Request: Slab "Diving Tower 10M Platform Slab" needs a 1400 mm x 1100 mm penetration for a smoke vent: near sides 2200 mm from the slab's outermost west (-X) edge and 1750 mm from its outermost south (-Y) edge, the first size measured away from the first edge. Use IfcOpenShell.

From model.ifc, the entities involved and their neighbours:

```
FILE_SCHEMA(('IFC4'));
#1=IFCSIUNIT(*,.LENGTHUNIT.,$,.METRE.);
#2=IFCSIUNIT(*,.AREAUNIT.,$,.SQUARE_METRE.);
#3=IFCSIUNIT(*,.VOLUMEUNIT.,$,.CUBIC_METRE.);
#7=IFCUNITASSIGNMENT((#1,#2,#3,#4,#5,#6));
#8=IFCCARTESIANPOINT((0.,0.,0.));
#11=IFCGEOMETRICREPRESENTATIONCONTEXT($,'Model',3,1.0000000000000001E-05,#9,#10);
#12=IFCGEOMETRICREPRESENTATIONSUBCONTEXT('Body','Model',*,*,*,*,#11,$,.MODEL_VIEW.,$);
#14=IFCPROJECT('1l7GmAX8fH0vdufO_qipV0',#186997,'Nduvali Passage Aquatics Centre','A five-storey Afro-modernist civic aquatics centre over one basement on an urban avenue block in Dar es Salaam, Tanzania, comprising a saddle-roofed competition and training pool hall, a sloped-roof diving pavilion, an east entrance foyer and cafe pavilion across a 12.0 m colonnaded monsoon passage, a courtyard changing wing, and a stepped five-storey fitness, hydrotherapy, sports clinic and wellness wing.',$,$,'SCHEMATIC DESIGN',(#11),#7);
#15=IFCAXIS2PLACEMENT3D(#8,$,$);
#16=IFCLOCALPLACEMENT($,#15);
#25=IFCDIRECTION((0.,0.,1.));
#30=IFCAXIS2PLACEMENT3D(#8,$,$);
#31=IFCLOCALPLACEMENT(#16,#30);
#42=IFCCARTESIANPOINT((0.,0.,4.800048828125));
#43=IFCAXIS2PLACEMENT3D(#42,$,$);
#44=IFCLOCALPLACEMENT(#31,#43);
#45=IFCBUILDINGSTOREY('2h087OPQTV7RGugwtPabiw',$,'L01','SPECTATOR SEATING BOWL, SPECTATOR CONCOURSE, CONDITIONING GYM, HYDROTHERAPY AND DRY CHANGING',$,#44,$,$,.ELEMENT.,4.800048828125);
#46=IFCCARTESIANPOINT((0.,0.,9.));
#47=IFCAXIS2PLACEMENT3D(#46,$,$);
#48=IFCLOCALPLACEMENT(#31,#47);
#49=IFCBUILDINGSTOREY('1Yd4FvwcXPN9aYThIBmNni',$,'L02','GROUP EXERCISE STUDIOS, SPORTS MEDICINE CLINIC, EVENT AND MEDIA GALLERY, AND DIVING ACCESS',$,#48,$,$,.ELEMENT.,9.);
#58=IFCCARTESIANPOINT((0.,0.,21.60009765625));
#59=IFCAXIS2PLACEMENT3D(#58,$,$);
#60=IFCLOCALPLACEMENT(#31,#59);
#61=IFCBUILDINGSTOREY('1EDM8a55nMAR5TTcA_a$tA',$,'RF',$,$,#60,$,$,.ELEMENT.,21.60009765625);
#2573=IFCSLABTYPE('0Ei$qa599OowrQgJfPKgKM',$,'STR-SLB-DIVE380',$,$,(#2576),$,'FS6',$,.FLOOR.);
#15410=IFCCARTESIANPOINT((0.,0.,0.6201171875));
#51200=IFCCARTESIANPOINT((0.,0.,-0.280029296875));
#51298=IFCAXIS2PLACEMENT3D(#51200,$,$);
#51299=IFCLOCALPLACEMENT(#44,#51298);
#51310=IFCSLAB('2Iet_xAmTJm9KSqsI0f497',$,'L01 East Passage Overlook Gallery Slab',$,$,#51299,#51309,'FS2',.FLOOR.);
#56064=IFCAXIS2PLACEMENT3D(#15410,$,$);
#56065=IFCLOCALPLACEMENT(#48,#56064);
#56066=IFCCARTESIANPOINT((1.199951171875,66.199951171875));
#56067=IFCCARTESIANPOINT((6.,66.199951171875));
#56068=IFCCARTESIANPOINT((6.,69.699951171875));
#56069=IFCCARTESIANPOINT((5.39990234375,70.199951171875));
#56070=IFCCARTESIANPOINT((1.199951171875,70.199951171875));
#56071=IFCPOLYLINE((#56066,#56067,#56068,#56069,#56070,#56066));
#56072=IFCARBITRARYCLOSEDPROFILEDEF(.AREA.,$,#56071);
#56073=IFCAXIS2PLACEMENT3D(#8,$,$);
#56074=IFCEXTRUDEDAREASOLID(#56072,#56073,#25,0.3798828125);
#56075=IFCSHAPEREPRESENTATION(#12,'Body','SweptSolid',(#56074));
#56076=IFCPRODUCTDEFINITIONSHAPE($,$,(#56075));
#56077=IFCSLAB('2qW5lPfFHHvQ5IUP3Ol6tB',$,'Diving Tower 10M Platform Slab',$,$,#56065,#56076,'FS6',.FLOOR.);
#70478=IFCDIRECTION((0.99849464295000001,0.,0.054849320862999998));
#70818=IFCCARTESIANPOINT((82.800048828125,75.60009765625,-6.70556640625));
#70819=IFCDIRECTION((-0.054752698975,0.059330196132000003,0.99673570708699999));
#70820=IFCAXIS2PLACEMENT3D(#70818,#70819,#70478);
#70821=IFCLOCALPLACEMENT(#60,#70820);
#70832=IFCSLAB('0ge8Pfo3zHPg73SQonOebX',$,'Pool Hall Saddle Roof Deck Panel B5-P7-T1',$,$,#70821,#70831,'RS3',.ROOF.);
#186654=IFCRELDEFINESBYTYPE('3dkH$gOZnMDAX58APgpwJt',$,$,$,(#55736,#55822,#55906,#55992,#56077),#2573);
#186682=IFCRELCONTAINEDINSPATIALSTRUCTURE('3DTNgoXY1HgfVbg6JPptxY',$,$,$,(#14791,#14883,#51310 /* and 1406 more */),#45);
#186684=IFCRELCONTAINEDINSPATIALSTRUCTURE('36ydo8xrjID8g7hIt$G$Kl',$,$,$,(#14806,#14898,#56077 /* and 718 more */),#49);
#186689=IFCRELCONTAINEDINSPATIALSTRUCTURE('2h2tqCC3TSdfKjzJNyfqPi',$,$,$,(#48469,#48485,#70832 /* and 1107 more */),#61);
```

```python
import numpy as np
import ifcopenshell
import ifcopenshell.api.feature
import ifcopenshell.api.geometry
import ifcopenshell.api.root
import ifcopenshell.geom
import ifcopenshell.util.placement
import ifcopenshell.util.representation
import ifcopenshell.util.shape
import ifcopenshell.util.unit

model = ifcopenshell.open("model.ifc")
unit_scale = ifcopenshell.util.unit.calculate_unit_scale(model)
settings = ifcopenshell.geom.settings()


def volume(element):
    """Net volume in cubic metres, openings subtracted."""
    shape = ifcopenshell.geom.create_shape(settings, element)
    return ifcopenshell.util.shape.get_volume(shape.geometry)


slab = model.by_guid("2qW5lPfFHHvQ5IUP3Ol6tB")
before = volume(slab)

# Extent in the slab's own axes, in metres. The edges named are its -X and -Y sides.
slab_shape = ifcopenshell.geom.create_shape(settings, slab)
vertices = ifcopenshell.util.shape.get_vertices(slab_shape.geometry)
x_min, y_min, bottom = vertices.min(axis=0)
top = vertices[:, 2].max()

opening = ifcopenshell.api.root.create_entity(model, ifc_class="IfcOpeningElement", name="Smoke vent opening", predefined_type="OPENING")
context = ifcopenshell.util.representation.get_context(model, "Model", "Body", "MODEL_VIEW")
width, depth = 1.4, 1.1
outline = [(0.0, 0.0), (width, 0.0), (width, depth), (0.0, depth), (0.0, 0.0)]
# Overshoot both faces by 50 mm so the cut is clean.
shape = ifcopenshell.api.geometry.add_slab_representation(
    model, context=context, depth=top - bottom + 0.1, polyline=outline
)
ifcopenshell.api.geometry.assign_representation(model, product=opening, representation=shape)

matrix = ifcopenshell.util.placement.get_local_placement(slab.ObjectPlacement)
matrix[:, 3] = matrix @ np.append(np.array([x_min + 2.2, y_min + 1.75, bottom - 0.05]) / unit_scale, 1.0)
ifcopenshell.api.geometry.edit_object_placement(model, product=opening, matrix=matrix, is_si=False)
ifcopenshell.api.feature.add_feature(model, feature=opening, element=slab)

after = volume(slab)

print(f"slab volume {before:.3f} -> {after:.3f} m3")

model.write("model-out.ifc")
```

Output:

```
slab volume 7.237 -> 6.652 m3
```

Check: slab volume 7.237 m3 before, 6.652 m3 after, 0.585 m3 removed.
